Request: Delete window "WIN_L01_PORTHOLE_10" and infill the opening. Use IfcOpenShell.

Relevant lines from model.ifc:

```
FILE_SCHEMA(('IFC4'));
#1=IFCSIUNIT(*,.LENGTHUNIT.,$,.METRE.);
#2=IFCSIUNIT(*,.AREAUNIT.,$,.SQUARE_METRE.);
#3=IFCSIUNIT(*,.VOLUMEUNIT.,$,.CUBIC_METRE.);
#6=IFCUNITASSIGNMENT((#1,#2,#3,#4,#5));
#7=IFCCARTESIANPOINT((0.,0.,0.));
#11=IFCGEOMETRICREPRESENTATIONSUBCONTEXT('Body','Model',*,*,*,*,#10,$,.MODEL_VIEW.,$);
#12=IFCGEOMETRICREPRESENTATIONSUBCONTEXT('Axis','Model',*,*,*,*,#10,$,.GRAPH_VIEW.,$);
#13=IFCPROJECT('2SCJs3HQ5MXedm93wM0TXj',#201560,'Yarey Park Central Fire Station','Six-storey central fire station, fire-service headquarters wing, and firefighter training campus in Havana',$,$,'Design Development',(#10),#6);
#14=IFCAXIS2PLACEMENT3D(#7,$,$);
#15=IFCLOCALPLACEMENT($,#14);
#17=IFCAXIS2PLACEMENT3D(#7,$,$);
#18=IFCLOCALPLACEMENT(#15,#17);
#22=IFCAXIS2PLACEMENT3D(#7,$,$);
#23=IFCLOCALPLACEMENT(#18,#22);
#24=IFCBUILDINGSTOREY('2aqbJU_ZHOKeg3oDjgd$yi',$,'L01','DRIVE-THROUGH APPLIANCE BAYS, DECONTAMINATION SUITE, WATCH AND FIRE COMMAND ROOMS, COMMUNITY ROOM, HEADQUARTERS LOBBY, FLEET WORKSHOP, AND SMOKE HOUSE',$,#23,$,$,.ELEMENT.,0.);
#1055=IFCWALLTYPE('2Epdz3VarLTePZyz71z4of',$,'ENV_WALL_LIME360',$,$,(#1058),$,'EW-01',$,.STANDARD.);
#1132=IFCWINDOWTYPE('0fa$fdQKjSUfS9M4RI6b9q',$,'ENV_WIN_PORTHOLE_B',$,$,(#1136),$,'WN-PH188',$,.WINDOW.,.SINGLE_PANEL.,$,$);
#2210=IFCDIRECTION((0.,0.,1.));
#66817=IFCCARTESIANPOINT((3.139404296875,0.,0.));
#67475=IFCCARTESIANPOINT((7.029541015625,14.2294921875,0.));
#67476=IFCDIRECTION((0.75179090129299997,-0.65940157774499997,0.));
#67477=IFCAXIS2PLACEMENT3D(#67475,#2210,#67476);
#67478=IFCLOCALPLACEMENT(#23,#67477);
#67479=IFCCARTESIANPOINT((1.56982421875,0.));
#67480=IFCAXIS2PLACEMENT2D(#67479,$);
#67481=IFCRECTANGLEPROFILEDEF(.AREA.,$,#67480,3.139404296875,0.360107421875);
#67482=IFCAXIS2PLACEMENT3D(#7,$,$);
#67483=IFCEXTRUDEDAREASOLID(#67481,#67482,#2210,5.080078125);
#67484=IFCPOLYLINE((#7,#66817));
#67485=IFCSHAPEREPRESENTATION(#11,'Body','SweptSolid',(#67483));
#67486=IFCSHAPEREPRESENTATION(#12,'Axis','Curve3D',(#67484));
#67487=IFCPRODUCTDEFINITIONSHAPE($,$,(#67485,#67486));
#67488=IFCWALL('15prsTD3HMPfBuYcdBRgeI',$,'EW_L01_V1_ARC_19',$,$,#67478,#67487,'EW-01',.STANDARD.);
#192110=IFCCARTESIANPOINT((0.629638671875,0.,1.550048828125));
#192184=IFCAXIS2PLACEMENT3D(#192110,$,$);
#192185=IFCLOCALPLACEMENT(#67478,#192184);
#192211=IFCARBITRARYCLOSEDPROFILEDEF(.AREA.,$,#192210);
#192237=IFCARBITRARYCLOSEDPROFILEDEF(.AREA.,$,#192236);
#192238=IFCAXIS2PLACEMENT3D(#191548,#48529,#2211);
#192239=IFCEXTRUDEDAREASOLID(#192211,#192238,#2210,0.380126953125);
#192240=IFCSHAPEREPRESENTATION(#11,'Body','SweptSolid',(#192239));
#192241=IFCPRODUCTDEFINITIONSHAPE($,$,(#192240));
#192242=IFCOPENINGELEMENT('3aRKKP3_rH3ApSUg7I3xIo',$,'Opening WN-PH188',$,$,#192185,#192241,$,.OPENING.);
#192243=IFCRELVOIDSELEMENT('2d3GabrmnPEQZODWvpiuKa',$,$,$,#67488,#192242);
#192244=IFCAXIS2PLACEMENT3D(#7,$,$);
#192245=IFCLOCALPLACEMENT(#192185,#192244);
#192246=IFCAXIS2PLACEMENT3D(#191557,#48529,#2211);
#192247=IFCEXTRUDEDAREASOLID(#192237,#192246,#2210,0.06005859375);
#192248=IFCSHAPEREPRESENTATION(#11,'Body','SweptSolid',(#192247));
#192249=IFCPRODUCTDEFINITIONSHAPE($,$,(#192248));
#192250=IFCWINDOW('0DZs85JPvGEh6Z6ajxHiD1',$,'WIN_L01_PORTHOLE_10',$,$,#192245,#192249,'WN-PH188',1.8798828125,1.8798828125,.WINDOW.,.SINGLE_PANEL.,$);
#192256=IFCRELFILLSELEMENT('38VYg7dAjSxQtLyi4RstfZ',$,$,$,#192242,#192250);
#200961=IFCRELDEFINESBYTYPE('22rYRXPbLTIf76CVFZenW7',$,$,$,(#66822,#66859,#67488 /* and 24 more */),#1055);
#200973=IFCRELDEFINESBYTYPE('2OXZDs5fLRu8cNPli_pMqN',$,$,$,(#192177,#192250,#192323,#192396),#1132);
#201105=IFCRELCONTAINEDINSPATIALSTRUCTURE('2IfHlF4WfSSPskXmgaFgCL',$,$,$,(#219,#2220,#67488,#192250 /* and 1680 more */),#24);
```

```python
import ifcopenshell
import ifcopenshell.api.feature
import ifcopenshell.api.root
import ifcopenshell.geom
import ifcopenshell.util.shape

model = ifcopenshell.open("model.ifc")
settings = ifcopenshell.geom.settings()


def volume(element):
    """Net volume in cubic metres, openings subtracted."""
    shape = ifcopenshell.geom.create_shape(settings, element)
    return ifcopenshell.util.shape.get_volume(shape.geometry)


window = model.by_guid("0DZs85JPvGEh6Z6ajxHiD1")
opening = window.FillsVoids[0].RelatingOpeningElement
wall = opening.VoidsElements[0].RelatingBuildingElement
before = volume(wall)

ifcopenshell.api.root.remove_product(model, product=window)
ifcopenshell.api.feature.remove_feature(model, feature=opening)

after = volume(wall)

print(f"wall volume {before:.3f} -> {after:.3f} m3")

model.write("model_rev.ifc")
```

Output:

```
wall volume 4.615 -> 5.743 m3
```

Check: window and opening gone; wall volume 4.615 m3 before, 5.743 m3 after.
